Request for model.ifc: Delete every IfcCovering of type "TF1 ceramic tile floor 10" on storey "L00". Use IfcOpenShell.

First a look at what the model holds.

```python
import ifcopenshell
import ifcopenshell.util.element

model = ifcopenshell.open("model.ifc")
print(model.schema)
storey = next(s for s in model.by_type("IfcBuildingStorey") if s.Name == "L00")
coverings = [e for e in ifcopenshell.util.element.get_decomposition(storey) if e.is_a("IfcCovering")]
seen = {}
for e in coverings:
    element_type = ifcopenshell.util.element.get_type(e)
    name = element_type.Name if element_type not in (None, e) else None
    seen[name] = seen.get(name, 0) + 1
for name, count in sorted(seen.items(), key=str):
    print(count, "x", name)
```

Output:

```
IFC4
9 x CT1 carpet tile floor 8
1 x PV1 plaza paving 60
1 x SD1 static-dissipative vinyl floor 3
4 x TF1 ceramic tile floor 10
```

```python
import ifcopenshell
import ifcopenshell.api.root
import ifcopenshell.util.element

model = ifcopenshell.open("model.ifc")

storey = next(s for s in model.by_type("IfcBuildingStorey") if s.Name == "L00")
coverings = [e for e in ifcopenshell.util.element.get_decomposition(storey) if e.is_a("IfcCovering")]
targets = [e for e in coverings if (t := ifcopenshell.util.element.get_type(e)) not in (None, e) and t.Name == "TF1 ceramic tile floor 10"]

for e in targets:
    ifcopenshell.api.root.remove_product(model, product=e)
print(len(targets), "removed")

model.write("model_updated.ifc")
```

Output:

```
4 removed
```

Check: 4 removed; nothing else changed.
